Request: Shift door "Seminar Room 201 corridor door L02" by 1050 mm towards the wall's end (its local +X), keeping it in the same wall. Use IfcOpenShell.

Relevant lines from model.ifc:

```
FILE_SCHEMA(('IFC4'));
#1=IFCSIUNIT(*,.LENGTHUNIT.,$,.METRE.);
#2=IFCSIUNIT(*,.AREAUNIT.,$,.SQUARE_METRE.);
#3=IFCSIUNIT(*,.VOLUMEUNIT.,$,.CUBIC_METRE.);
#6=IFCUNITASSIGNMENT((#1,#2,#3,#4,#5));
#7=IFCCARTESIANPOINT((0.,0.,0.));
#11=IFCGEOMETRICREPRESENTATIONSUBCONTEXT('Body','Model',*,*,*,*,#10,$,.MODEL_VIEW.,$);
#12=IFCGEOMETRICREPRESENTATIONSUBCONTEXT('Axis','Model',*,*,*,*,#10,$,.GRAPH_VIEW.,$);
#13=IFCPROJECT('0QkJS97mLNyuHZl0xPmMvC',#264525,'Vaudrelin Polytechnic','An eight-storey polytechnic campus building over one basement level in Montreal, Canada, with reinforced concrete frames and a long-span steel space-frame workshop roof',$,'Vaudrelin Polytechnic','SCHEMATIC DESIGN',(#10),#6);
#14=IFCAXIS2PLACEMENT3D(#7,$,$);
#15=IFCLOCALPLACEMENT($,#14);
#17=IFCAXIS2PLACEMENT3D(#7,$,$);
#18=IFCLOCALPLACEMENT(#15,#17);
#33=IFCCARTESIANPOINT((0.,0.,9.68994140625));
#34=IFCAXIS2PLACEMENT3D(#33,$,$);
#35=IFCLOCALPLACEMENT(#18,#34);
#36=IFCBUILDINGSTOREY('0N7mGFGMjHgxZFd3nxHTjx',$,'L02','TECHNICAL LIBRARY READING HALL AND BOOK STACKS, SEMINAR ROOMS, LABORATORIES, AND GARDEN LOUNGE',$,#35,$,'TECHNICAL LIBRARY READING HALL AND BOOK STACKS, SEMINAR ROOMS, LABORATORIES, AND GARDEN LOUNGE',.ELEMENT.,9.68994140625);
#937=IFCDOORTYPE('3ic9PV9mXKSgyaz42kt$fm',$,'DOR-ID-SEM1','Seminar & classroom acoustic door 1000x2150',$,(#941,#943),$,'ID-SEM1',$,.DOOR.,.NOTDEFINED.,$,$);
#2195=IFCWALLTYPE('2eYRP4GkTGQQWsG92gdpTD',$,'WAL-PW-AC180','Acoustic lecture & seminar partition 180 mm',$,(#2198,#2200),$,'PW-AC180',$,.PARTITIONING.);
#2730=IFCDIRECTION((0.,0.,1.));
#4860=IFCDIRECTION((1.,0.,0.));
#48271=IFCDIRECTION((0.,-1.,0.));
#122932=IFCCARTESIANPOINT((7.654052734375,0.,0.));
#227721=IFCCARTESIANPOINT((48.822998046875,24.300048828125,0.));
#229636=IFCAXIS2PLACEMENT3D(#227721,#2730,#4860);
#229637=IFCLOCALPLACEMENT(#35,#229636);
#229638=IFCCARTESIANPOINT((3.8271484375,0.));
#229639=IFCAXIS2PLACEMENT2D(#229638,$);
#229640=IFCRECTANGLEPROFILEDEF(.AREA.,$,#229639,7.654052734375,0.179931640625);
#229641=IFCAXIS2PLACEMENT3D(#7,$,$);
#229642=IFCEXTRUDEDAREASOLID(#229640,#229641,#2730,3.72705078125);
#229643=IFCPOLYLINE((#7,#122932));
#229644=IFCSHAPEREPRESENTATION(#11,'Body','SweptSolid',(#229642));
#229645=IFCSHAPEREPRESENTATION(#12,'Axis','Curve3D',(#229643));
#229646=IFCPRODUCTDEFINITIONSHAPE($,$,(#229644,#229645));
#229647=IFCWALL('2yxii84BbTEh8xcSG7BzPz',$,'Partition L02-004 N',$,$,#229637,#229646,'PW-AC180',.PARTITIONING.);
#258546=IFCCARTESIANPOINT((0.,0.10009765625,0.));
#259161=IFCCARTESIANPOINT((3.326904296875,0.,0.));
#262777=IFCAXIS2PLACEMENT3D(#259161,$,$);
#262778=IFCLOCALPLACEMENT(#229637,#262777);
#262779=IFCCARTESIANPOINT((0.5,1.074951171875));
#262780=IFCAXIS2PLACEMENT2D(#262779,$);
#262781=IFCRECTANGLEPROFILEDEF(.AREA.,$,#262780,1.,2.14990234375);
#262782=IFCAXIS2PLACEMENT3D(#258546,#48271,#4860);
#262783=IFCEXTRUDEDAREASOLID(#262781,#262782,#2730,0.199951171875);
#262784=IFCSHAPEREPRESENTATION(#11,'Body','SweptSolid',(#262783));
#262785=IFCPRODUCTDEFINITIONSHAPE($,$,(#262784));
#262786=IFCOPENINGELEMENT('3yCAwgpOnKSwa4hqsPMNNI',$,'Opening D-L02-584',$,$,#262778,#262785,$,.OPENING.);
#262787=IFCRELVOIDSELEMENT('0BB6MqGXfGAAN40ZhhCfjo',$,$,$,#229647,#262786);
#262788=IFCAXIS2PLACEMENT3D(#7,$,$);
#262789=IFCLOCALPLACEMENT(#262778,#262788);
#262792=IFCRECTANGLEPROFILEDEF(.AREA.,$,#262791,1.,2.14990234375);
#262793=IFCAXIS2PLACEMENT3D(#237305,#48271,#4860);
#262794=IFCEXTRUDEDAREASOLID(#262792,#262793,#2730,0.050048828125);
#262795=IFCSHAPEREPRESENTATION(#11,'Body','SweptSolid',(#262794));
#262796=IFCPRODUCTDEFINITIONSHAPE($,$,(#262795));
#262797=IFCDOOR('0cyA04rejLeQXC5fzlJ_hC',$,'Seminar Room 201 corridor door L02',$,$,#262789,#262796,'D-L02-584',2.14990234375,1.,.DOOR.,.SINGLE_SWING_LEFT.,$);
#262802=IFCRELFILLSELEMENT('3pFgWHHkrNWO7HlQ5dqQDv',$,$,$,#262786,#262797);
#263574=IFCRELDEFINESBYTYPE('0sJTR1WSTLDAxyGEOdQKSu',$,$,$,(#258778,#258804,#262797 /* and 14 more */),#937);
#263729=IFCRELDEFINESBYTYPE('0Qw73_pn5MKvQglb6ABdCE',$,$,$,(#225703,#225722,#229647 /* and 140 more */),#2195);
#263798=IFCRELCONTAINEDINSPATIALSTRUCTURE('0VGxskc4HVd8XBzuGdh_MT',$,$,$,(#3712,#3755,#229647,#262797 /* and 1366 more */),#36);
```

```python
import ifcopenshell
import ifcopenshell.api.geometry
import ifcopenshell.util.placement

model = ifcopenshell.open("model.ifc")

door = model.by_guid("0cyA04rejLeQXC5fzlJ_hC")
opening = door.FillsVoids[0].RelatingOpeningElement
wall = opening.VoidsElements[0].RelatingBuildingElement

wall_matrix = ifcopenshell.util.placement.get_local_placement(wall.ObjectPlacement)
shift = wall_matrix[:3, 0] * 1.05
before = ifcopenshell.util.placement.get_local_placement(door.ObjectPlacement)[:3, 3].copy()

# The door is placed relative to its opening, so it follows when the opening moves.
matrix = ifcopenshell.util.placement.get_local_placement(opening.ObjectPlacement)
matrix[:3, 3] += shift
ifcopenshell.api.geometry.edit_object_placement(
    model, product=opening, matrix=matrix, is_si=False, should_transform_children=True
)

after = ifcopenshell.util.placement.get_local_placement(door.ObjectPlacement)[:3, 3]
print("door moved by", (after - before).round(3) + 0.0)

model.write("model_updated.ifc")
```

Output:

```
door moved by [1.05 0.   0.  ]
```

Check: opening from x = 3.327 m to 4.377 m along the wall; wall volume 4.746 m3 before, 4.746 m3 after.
